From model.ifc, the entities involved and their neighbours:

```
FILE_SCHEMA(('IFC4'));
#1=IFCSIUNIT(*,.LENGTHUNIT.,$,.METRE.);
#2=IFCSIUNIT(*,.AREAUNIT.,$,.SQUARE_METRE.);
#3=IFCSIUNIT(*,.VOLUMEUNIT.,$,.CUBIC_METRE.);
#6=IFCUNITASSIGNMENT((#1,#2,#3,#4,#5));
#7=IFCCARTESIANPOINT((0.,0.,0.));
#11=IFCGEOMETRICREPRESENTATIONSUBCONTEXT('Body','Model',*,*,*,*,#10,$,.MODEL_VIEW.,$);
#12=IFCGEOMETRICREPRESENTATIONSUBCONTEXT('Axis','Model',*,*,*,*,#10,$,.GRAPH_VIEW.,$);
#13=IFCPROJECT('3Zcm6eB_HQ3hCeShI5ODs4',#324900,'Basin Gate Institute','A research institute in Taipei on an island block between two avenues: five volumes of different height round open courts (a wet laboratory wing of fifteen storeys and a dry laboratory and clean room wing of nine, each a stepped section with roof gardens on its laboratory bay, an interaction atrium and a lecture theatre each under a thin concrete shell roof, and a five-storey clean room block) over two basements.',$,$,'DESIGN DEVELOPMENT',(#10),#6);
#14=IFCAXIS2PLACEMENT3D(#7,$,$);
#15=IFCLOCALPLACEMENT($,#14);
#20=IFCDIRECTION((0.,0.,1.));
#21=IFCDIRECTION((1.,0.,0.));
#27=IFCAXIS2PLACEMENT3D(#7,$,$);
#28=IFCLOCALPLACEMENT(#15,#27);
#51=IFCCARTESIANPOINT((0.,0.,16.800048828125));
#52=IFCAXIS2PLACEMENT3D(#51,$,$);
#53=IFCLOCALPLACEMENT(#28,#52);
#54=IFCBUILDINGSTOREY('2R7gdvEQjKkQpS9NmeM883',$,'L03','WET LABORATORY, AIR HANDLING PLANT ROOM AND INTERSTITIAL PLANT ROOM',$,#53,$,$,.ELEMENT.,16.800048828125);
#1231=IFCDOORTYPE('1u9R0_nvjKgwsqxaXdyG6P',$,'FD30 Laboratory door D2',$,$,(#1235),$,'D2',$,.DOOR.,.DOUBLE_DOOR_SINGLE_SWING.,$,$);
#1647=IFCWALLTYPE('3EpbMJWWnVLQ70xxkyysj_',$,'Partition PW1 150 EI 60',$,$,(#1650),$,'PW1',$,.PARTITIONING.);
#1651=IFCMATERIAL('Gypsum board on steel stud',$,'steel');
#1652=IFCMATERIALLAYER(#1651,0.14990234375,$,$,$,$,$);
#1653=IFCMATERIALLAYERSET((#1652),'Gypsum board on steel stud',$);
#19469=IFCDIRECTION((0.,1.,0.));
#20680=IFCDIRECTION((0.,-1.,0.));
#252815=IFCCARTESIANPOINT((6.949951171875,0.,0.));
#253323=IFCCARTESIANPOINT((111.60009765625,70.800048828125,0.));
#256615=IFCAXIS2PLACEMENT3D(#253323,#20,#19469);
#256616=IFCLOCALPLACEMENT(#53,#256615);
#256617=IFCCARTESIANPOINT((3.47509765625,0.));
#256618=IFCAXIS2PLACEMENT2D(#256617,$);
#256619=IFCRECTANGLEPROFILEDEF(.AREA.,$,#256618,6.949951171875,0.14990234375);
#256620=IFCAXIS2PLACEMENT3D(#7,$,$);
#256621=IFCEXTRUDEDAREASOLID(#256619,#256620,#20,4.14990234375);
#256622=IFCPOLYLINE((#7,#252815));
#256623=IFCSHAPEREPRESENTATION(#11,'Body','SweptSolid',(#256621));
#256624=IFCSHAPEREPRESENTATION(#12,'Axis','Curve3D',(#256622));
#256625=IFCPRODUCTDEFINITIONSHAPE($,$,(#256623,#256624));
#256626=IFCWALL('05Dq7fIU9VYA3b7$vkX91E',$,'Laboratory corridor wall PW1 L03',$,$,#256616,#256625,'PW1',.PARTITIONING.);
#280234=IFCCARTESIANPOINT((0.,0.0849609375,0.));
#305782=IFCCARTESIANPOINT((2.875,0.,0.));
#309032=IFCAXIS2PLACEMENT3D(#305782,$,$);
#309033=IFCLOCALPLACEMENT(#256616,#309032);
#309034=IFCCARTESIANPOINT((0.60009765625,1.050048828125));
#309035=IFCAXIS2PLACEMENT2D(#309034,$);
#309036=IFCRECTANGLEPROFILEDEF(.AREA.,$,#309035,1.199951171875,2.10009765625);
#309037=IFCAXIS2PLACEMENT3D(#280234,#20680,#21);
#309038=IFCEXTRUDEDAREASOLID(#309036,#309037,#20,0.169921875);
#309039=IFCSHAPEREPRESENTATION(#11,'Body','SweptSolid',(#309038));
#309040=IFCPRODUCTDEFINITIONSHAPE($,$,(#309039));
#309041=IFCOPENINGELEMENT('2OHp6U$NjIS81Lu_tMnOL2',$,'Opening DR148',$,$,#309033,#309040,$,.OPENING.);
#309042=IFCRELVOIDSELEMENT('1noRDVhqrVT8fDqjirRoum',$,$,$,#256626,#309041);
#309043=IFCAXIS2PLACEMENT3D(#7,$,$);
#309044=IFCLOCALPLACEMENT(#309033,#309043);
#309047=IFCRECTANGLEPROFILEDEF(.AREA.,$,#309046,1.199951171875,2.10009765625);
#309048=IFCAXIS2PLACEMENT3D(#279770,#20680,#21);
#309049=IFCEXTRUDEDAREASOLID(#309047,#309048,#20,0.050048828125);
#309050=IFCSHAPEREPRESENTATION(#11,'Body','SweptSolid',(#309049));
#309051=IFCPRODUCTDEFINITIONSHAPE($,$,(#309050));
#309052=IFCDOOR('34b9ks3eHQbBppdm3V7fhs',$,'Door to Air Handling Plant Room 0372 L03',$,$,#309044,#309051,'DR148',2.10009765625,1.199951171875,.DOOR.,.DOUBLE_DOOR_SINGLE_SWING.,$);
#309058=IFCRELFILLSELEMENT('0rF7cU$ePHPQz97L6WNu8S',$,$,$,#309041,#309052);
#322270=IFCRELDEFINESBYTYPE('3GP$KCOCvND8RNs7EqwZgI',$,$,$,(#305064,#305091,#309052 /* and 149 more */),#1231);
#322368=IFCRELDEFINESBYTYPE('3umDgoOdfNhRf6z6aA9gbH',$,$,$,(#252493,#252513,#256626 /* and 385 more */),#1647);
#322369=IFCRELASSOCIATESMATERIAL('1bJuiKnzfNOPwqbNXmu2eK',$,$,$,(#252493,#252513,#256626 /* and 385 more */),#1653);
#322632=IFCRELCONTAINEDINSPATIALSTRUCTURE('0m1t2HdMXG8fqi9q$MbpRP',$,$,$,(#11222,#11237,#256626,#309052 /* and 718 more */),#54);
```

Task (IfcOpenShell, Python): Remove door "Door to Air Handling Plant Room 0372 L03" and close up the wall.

```python
import ifcopenshell
import ifcopenshell.api.feature
import ifcopenshell.api.root
import ifcopenshell.geom
import ifcopenshell.util.shape

model = ifcopenshell.open("model.ifc")
settings = ifcopenshell.geom.settings()


def volume(element):
    """Net volume in cubic metres, openings subtracted."""
    shape = ifcopenshell.geom.create_shape(settings, element)
    return ifcopenshell.util.shape.get_volume(shape.geometry)


door = model.by_id(309052)
opening = door.FillsVoids[0].RelatingOpeningElement
wall = opening.VoidsElements[0].RelatingBuildingElement
before = volume(wall)

ifcopenshell.api.root.remove_product(model, product=door)
ifcopenshell.api.feature.remove_feature(model, feature=opening)

after = volume(wall)

print(f"wall volume {before:.3f} -> {after:.3f} m3")

model.write("model_rev.ifc")
```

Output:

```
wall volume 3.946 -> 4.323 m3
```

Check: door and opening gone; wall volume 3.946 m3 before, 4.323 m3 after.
